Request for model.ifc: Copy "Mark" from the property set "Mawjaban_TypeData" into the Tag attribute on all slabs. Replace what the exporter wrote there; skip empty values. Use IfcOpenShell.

First a look at what the model holds.

```python
import ifcopenshell
import ifcopenshell.util.element

model = ifcopenshell.open("model.ifc")
print(model.schema)
slabs = model.by_type("IfcSlab")
print(len(slabs), "slabs")
for e in slabs[:8]:
    source = ifcopenshell.util.element.get_pset(e, "Mawjaban_TypeData", "Mark")
    target = e.Tag
    print(e.id(), repr(source), repr(target), sep=" | ")
```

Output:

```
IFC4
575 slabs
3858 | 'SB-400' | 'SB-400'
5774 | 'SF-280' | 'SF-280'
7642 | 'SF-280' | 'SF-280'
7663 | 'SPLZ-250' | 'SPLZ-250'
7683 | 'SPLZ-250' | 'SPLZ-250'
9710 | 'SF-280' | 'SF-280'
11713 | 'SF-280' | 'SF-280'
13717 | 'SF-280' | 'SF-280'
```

```python
import ifcopenshell
import ifcopenshell.util.element

model = ifcopenshell.open("model.ifc")

count = 0
for e in model.by_type("IfcSlab"):
    value = ifcopenshell.util.element.get_pset(e, "Mawjaban_TypeData", "Mark")
    current = e.Tag
    if not value or not value.strip() or current == value:
        continue
    e.Tag = value
    count += 1

print(count, "slabs updated")

model.write("model_updated.ifc")
```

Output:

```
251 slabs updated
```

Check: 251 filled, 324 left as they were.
